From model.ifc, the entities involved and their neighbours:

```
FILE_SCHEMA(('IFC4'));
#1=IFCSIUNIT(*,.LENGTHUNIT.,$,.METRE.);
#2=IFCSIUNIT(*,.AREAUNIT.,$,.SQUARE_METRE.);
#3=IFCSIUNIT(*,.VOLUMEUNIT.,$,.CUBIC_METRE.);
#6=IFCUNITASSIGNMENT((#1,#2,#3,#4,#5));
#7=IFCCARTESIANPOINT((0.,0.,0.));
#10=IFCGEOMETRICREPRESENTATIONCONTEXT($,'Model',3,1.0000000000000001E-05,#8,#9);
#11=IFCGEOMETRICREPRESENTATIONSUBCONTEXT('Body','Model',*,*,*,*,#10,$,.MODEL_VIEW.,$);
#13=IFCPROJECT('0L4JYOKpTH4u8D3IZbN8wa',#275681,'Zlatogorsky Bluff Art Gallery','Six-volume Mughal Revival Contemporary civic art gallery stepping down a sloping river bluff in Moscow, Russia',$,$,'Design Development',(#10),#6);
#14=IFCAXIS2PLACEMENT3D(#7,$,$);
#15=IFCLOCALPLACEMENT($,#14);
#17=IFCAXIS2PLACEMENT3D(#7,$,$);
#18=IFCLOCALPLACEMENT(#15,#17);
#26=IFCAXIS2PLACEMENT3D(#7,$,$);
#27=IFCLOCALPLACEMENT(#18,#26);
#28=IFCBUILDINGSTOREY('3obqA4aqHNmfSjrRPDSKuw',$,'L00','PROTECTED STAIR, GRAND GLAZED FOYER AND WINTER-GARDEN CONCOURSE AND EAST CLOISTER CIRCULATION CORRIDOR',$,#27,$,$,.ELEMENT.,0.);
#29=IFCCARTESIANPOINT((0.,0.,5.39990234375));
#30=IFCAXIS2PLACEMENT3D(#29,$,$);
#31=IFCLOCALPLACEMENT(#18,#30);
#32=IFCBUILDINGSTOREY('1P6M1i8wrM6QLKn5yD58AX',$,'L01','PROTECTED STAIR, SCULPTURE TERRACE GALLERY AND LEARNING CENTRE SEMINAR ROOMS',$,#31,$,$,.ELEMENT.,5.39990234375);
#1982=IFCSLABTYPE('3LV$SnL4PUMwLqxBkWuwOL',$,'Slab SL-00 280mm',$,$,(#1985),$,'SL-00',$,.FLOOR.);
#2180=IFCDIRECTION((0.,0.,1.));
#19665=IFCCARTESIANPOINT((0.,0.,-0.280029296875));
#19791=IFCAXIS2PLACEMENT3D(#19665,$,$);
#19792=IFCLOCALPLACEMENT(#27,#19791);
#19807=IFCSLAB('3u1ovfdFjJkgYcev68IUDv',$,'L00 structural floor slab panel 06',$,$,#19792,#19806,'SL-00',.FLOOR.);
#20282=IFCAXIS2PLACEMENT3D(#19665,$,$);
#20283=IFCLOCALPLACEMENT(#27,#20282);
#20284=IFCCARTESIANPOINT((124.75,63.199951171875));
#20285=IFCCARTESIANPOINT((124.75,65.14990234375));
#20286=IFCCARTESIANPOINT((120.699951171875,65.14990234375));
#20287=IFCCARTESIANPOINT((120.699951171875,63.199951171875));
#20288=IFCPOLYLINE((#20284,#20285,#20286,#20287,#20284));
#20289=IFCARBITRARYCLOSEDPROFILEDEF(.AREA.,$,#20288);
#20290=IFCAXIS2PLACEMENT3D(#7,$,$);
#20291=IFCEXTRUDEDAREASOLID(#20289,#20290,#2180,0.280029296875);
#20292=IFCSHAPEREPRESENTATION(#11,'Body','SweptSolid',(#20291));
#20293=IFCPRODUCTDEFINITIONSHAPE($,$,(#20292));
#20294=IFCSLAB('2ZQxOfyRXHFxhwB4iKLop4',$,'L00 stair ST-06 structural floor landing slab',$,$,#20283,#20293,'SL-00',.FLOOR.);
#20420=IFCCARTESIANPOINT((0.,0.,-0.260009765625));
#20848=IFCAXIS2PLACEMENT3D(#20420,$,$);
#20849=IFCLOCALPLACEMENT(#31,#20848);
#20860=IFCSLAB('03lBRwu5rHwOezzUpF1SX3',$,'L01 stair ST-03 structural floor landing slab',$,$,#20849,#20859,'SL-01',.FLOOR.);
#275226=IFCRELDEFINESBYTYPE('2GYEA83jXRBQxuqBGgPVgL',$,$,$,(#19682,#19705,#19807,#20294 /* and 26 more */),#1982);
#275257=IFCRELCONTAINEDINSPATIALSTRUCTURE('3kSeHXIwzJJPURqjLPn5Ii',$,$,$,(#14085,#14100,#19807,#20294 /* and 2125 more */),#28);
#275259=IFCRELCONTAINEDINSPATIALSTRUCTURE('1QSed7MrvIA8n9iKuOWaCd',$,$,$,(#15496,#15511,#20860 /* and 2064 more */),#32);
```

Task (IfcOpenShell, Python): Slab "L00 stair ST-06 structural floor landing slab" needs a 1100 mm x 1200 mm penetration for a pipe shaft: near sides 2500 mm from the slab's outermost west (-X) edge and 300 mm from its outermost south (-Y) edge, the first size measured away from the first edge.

```python
import numpy as np
import ifcopenshell
import ifcopenshell.api.feature
import ifcopenshell.api.geometry
import ifcopenshell.api.root
import ifcopenshell.geom
import ifcopenshell.util.placement
import ifcopenshell.util.representation
import ifcopenshell.util.shape
import ifcopenshell.util.unit

model = ifcopenshell.open("model.ifc")
unit_scale = ifcopenshell.util.unit.calculate_unit_scale(model)
settings = ifcopenshell.geom.settings()


def volume(element):
    """Net volume in cubic metres, openings subtracted."""
    shape = ifcopenshell.geom.create_shape(settings, element)
    return ifcopenshell.util.shape.get_volume(shape.geometry)


slab = model.by_guid("2ZQxOfyRXHFxhwB4iKLop4")
before = volume(slab)

# Extent in the slab's own axes, in metres. The edges named are its -X and -Y sides.
slab_shape = ifcopenshell.geom.create_shape(settings, slab)
vertices = ifcopenshell.util.shape.get_vertices(slab_shape.geometry)
x_min, y_min, bottom = vertices.min(axis=0)
top = vertices[:, 2].max()

opening = ifcopenshell.api.root.create_entity(model, ifc_class="IfcOpeningElement", name="Pipe shaft opening", predefined_type="OPENING")
context = ifcopenshell.util.representation.get_context(model, "Model", "Body", "MODEL_VIEW")
width, depth = 1.1, 1.2
outline = [(0.0, 0.0), (width, 0.0), (width, depth), (0.0, depth), (0.0, 0.0)]
# Overshoot both faces by 50 mm so the cut is clean.
shape = ifcopenshell.api.geometry.add_slab_representation(
    model, context=context, depth=top - bottom + 0.1, polyline=outline
)
ifcopenshell.api.geometry.assign_representation(model, product=opening, representation=shape)

matrix = ifcopenshell.util.placement.get_local_placement(slab.ObjectPlacement)
matrix[:, 3] = matrix @ np.append(np.array([x_min + 2.5, y_min + 0.3, bottom - 0.05]) / unit_scale, 1.0)
ifcopenshell.api.geometry.edit_object_placement(model, product=opening, matrix=matrix, is_si=False)
ifcopenshell.api.feature.add_feature(model, feature=opening, element=slab)

after = volume(slab)

print(f"slab volume {before:.3f} -> {after:.3f} m3")

model.write("model_v2.ifc")
```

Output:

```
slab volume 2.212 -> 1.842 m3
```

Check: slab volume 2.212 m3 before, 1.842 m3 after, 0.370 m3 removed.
